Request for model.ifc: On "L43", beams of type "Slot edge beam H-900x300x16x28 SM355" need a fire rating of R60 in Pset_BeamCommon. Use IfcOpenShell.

First a look at what the model holds.

```python
import ifcopenshell
import ifcopenshell.util.element

model = ifcopenshell.open("model.ifc")
print(model.schema)
storey = next(s for s in model.by_type("IfcBuildingStorey") if s.Name == "L43")
beams = [e for e in ifcopenshell.util.element.get_decomposition(storey) if e.is_a("IfcBeam")]
seen = {}
for e in beams:
    element_type = ifcopenshell.util.element.get_type(e)
    key = (element_type.Name if element_type != e and element_type else None, ifcopenshell.util.element.get_pset(e, "Pset_BeamCommon", "FireRating"))
    seen[key] = seen.get(key, 0) + 1
for (name, value), count in sorted(seen.items(), key=str):
    print(count, "x", name, "|", value)
```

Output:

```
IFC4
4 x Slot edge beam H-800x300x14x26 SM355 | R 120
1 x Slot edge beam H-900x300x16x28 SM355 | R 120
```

```python
import ifcopenshell
import ifcopenshell.api.pset
import ifcopenshell.util.element

model = ifcopenshell.open("model.ifc")

storey = next(s for s in model.by_type("IfcBuildingStorey") if s.Name == "L43")
beams = [e for e in ifcopenshell.util.element.get_decomposition(storey) if e.is_a("IfcBeam")]

count = 0
for e in beams:
    element_type = ifcopenshell.util.element.get_type(e)
    if element_type in (None, e) or element_type.Name != "Slot edge beam H-900x300x16x28 SM355":
        continue
    # add_pset returns the element's existing set when there is one.
    pset = ifcopenshell.api.pset.add_pset(model, product=e, name="Pset_BeamCommon")
    ifcopenshell.api.pset.edit_pset(model, pset=pset, properties={"FireRating": "R60"})
    count += 1

print(count, "beams updated")

model.write("model_rev.ifc")
```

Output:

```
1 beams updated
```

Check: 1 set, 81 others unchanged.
